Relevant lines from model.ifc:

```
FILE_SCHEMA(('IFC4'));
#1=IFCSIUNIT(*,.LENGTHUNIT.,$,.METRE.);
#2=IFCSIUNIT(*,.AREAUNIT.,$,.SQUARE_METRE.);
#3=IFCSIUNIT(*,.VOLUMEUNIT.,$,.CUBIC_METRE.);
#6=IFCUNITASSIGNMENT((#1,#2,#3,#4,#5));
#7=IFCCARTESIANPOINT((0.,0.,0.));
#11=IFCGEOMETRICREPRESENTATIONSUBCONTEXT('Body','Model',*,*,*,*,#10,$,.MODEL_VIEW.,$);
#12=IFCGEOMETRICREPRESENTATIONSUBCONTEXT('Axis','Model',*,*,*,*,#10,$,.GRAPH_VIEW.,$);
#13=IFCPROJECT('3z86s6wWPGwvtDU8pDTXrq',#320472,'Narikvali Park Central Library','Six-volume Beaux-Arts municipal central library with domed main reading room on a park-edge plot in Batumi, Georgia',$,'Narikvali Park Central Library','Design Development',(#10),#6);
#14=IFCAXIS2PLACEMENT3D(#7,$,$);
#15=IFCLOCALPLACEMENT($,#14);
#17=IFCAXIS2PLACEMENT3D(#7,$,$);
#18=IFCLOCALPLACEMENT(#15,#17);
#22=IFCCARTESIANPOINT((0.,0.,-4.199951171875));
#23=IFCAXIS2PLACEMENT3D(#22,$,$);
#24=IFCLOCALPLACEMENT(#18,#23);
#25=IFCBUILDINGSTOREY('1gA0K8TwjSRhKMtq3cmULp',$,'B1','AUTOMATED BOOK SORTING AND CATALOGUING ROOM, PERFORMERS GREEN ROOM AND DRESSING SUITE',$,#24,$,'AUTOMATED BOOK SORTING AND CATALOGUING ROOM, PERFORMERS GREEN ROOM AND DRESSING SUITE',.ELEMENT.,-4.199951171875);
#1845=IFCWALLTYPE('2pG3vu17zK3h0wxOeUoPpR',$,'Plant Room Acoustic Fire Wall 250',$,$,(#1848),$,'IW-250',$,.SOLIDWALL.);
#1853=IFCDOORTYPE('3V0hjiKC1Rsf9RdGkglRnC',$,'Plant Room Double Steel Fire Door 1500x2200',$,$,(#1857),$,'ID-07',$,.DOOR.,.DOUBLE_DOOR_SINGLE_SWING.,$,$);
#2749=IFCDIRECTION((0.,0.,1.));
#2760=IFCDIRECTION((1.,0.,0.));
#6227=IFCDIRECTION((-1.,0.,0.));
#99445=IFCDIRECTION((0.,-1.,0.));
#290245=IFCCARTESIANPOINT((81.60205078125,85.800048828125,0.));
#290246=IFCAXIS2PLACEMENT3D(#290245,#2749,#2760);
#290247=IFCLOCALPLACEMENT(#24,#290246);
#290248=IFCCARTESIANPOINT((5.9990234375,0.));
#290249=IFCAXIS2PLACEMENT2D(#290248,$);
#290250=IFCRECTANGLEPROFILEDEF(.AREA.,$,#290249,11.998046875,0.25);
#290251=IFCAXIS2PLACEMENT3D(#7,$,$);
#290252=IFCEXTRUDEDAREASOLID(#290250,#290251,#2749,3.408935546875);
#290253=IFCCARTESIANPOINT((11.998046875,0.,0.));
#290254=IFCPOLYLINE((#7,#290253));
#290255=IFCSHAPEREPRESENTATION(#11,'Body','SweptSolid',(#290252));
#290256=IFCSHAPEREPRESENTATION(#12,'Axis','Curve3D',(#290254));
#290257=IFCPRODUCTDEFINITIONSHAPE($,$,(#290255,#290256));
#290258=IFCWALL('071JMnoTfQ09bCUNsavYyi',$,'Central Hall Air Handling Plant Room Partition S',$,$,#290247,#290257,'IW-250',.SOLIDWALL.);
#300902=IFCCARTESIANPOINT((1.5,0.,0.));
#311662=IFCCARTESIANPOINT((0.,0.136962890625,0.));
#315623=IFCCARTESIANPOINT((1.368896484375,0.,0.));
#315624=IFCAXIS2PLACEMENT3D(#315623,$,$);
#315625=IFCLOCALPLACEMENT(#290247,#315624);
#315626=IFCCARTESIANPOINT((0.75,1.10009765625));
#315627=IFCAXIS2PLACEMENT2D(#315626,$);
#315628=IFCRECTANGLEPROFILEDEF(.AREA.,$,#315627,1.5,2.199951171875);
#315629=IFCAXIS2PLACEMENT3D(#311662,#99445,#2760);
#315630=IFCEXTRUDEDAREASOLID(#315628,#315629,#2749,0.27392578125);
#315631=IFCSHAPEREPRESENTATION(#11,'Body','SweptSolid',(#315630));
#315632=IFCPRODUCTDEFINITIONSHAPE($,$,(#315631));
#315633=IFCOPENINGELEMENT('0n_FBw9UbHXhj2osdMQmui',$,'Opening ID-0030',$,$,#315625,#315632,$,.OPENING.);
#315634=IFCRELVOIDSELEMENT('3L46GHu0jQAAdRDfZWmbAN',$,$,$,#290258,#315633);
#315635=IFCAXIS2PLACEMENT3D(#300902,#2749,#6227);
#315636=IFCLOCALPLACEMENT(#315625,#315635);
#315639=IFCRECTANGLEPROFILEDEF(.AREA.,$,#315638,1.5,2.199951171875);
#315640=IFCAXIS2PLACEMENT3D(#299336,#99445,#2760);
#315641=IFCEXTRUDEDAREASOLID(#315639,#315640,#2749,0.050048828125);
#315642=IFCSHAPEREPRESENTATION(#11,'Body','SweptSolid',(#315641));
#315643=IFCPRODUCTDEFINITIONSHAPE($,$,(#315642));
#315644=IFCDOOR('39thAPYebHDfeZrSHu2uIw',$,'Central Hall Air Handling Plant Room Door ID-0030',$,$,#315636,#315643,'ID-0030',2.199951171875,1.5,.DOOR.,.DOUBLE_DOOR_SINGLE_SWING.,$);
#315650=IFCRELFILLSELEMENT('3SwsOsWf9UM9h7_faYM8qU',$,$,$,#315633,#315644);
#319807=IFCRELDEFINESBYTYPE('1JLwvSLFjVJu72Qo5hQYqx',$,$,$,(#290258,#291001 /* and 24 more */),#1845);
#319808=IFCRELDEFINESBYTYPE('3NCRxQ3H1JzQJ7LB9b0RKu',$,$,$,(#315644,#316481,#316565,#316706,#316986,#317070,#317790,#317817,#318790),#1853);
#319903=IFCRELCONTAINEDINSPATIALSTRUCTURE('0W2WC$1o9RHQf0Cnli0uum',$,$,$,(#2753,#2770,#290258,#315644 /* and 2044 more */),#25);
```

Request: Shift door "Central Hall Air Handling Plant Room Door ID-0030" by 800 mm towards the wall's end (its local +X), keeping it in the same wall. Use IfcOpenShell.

```python
import ifcopenshell
import ifcopenshell.api.geometry
import ifcopenshell.util.placement

model = ifcopenshell.open("model.ifc")

door = model.by_guid("39thAPYebHDfeZrSHu2uIw")
opening = door.FillsVoids[0].RelatingOpeningElement
wall = opening.VoidsElements[0].RelatingBuildingElement

wall_matrix = ifcopenshell.util.placement.get_local_placement(wall.ObjectPlacement)
shift = wall_matrix[:3, 0] * 0.8
before = ifcopenshell.util.placement.get_local_placement(door.ObjectPlacement)[:3, 3].copy()

# The door is placed relative to its opening, so it follows when the opening moves.
matrix = ifcopenshell.util.placement.get_local_placement(opening.ObjectPlacement)
matrix[:3, 3] += shift
ifcopenshell.api.geometry.edit_object_placement(
    model, product=opening, matrix=matrix, is_si=False, should_transform_children=True
)

after = ifcopenshell.util.placement.get_local_placement(door.ObjectPlacement)[:3, 3]
print("door moved by", (after - before).round(3) + 0.0)

model.write("model-out.ifc")
```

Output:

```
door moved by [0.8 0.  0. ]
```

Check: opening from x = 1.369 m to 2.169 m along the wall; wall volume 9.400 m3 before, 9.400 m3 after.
